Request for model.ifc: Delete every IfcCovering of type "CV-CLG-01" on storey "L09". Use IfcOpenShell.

First a look at what the model holds.

```python
import ifcopenshell
import ifcopenshell.util.element

model = ifcopenshell.open("model.ifc")
print(model.schema)
storey = next(s for s in model.by_type("IfcBuildingStorey") if s.Name == "L09")
coverings = [e for e in ifcopenshell.util.element.get_decomposition(storey) if e.is_a("IfcCovering")]
seen = {}
for e in coverings:
    element_type = ifcopenshell.util.element.get_type(e)
    name = element_type.Name if element_type not in (None, e) else None
    seen[name] = seen.get(name, 0) + 1
for name, count in sorted(seen.items(), key=str):
    print(count, "x", name)
```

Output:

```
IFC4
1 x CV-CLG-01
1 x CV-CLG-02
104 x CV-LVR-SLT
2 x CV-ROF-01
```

```python
import ifcopenshell
import ifcopenshell.api.root
import ifcopenshell.util.element

model = ifcopenshell.open("model.ifc")

storey = next(s for s in model.by_type("IfcBuildingStorey") if s.Name == "L09")
coverings = [e for e in ifcopenshell.util.element.get_decomposition(storey) if e.is_a("IfcCovering")]
targets = [e for e in coverings if (t := ifcopenshell.util.element.get_type(e)) not in (None, e) and t.Name == "CV-CLG-01"]

for e in targets:
    ifcopenshell.api.root.remove_product(model, product=e)
print(len(targets), "removed")

model.write("model_updated.ifc")
```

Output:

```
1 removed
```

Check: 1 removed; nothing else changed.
